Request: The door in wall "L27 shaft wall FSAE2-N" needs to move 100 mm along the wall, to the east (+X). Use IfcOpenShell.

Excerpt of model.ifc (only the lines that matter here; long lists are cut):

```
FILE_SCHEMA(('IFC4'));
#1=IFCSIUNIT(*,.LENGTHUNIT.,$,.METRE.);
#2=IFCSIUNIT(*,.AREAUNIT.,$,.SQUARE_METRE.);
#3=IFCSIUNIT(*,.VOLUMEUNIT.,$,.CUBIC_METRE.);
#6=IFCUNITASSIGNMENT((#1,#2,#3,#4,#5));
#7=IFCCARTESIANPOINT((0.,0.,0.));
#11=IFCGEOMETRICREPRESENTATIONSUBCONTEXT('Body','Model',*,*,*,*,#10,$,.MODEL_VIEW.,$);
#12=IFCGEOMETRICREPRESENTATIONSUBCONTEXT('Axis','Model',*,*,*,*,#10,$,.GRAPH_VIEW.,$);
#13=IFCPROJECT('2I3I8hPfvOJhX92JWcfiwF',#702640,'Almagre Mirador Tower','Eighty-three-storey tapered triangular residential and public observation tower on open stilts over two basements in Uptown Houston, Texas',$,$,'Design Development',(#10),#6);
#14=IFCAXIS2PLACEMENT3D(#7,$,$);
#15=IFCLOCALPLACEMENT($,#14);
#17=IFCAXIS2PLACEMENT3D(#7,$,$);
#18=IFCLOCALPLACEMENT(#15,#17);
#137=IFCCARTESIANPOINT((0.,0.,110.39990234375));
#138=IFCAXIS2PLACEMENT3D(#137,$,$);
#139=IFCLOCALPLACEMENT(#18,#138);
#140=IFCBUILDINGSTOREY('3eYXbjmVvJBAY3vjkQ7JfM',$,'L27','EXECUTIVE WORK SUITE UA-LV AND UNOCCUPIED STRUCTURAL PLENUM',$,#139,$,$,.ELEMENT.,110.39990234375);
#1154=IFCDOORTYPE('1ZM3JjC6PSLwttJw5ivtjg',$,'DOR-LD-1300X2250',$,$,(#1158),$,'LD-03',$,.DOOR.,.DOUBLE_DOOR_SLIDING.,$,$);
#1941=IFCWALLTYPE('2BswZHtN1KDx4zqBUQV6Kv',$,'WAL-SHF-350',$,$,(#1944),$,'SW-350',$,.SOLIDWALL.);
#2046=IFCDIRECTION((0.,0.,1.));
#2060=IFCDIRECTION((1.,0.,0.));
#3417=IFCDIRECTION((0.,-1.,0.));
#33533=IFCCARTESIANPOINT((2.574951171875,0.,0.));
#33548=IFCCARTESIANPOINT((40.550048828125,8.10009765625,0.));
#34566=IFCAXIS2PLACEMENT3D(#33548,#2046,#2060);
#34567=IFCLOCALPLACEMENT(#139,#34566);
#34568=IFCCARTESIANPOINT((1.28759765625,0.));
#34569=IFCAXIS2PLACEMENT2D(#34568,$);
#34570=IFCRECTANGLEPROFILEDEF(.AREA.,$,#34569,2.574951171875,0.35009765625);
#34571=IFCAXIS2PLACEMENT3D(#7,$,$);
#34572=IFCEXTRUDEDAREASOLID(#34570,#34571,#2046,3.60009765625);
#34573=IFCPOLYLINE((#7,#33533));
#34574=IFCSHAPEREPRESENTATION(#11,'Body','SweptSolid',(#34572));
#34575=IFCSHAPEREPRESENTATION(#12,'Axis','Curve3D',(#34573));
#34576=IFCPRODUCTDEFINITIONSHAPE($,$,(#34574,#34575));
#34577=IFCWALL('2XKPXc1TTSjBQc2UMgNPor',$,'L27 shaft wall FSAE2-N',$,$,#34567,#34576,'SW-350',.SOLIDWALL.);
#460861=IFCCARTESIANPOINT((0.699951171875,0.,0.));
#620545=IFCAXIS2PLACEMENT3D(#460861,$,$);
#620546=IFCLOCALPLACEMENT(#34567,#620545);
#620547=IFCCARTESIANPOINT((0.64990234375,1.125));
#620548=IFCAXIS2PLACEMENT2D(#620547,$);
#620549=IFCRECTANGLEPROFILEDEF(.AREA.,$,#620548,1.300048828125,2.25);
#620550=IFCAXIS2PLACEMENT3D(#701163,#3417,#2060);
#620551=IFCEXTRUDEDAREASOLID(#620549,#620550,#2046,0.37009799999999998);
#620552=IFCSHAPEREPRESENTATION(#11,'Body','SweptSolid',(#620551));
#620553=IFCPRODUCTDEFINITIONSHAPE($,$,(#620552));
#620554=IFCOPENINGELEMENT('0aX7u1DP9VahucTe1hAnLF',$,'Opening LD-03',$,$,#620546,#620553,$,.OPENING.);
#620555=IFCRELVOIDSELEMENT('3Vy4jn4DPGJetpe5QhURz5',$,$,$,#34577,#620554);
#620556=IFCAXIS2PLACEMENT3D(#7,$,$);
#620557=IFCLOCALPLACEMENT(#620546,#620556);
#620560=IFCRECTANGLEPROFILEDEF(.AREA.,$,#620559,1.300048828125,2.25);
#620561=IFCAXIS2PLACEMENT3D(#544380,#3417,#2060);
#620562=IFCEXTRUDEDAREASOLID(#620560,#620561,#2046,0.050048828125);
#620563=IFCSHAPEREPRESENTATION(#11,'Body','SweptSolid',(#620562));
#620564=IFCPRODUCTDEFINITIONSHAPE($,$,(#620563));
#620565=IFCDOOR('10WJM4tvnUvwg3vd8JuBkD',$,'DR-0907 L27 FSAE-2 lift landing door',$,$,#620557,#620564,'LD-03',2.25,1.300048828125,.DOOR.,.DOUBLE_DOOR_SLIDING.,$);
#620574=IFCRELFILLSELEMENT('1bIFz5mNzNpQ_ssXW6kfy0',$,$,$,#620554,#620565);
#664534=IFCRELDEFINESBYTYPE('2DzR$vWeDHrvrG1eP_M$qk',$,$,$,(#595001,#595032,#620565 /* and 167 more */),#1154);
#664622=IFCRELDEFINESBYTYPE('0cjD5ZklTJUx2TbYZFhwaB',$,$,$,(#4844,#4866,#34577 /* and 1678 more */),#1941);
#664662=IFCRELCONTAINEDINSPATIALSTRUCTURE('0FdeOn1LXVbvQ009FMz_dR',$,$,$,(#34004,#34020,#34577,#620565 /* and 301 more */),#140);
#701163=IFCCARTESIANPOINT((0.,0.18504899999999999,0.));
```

```python
import ifcopenshell
import ifcopenshell.api.geometry
import ifcopenshell.util.placement

model = ifcopenshell.open("model.ifc")

door = model.by_guid("10WJM4tvnUvwg3vd8JuBkD")
opening = door.FillsVoids[0].RelatingOpeningElement
wall = opening.VoidsElements[0].RelatingBuildingElement

wall_matrix = ifcopenshell.util.placement.get_local_placement(wall.ObjectPlacement)
shift = wall_matrix[:3, 0] * 0.1
before = ifcopenshell.util.placement.get_local_placement(door.ObjectPlacement)[:3, 3].copy()

# The door is placed relative to its opening, so it follows when the opening moves.
matrix = ifcopenshell.util.placement.get_local_placement(opening.ObjectPlacement)
matrix[:3, 3] += shift
ifcopenshell.api.geometry.edit_object_placement(
    model, product=opening, matrix=matrix, is_si=False, should_transform_children=True
)

after = ifcopenshell.util.placement.get_local_placement(door.ObjectPlacement)[:3, 3]
print("door moved by", (after - before).round(3) + 0.0)

model.write("model_v2.ifc")
```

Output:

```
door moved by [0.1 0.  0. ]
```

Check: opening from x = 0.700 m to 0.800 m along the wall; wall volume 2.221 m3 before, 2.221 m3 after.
